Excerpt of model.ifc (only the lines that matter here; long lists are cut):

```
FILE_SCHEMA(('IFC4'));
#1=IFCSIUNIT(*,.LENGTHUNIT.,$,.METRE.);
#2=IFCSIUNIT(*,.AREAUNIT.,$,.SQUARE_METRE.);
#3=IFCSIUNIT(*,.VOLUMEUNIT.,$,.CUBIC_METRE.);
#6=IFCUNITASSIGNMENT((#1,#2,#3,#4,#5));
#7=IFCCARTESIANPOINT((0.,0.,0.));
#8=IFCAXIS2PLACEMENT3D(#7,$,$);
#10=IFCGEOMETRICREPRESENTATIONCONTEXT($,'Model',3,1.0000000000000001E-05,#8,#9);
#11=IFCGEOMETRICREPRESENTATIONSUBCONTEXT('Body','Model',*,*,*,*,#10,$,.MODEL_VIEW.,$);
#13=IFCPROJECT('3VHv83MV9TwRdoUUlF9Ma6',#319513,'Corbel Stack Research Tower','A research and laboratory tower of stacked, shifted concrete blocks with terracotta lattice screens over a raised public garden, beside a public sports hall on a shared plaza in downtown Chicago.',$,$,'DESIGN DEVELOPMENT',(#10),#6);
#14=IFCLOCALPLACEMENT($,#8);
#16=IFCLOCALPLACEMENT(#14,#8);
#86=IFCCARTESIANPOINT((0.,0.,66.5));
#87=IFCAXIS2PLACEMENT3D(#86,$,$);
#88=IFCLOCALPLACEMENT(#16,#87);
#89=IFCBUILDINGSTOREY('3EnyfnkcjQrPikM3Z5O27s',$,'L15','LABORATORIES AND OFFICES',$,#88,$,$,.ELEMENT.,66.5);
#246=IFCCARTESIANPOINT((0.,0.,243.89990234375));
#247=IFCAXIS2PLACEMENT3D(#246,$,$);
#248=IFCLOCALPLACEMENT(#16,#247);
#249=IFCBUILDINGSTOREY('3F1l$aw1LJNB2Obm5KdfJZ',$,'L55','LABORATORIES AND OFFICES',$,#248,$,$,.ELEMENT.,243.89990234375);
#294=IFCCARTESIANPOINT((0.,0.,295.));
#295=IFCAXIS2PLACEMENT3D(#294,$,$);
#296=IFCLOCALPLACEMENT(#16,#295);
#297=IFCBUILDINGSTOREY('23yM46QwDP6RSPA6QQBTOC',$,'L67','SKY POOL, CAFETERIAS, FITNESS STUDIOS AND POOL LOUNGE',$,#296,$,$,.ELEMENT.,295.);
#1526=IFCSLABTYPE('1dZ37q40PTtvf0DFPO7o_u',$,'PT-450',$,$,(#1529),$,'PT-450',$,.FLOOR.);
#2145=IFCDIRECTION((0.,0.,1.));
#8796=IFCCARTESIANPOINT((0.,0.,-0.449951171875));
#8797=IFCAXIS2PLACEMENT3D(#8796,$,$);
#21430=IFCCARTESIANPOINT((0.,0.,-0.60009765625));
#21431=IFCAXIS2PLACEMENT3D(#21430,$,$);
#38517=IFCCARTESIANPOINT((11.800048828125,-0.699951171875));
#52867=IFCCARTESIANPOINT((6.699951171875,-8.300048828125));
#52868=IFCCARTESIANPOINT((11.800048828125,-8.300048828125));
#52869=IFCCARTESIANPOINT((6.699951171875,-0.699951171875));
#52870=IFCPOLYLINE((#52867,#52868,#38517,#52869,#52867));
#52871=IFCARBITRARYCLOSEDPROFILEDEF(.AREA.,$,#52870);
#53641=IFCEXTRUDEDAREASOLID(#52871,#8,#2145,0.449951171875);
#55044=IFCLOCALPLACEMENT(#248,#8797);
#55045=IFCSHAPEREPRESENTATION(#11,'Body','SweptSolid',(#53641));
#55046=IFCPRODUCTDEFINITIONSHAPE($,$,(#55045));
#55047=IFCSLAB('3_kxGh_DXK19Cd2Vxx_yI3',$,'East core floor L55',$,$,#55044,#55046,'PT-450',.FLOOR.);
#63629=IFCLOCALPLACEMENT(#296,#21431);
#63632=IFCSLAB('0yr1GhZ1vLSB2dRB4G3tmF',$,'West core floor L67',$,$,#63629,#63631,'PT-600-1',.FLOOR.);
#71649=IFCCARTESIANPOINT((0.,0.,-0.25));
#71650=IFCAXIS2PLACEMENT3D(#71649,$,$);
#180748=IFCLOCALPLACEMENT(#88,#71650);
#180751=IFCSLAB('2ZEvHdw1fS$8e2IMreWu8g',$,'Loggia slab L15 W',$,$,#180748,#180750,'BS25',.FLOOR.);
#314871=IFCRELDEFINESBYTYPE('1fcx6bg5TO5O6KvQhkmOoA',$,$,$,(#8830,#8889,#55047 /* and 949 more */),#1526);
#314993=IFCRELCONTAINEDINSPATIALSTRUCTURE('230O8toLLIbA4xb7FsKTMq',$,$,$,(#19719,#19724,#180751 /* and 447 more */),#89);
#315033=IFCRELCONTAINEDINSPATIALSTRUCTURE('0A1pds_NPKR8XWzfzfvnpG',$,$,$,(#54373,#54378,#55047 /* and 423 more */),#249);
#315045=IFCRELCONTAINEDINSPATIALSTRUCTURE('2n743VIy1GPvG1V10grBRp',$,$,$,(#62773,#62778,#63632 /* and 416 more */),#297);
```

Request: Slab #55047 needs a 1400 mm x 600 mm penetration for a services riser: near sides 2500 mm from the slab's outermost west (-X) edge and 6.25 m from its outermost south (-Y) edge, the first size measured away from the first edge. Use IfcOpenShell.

```python
import numpy as np
import ifcopenshell
import ifcopenshell.api.feature
import ifcopenshell.api.geometry
import ifcopenshell.api.root
import ifcopenshell.geom
import ifcopenshell.util.placement
import ifcopenshell.util.representation
import ifcopenshell.util.shape
import ifcopenshell.util.unit

model = ifcopenshell.open("model.ifc")
unit_scale = ifcopenshell.util.unit.calculate_unit_scale(model)
settings = ifcopenshell.geom.settings()


def volume(element):
    """Net volume in cubic metres, openings subtracted."""
    shape = ifcopenshell.geom.create_shape(settings, element)
    return ifcopenshell.util.shape.get_volume(shape.geometry)


slab = model.by_guid("3_kxGh_DXK19Cd2Vxx_yI3")
before = volume(slab)

# Extent in the slab's own axes, in metres. The edges named are its -X and -Y sides.
slab_shape = ifcopenshell.geom.create_shape(settings, slab)
vertices = ifcopenshell.util.shape.get_vertices(slab_shape.geometry)
x_min, y_min, bottom = vertices.min(axis=0)
top = vertices[:, 2].max()

opening = ifcopenshell.api.root.create_entity(model, ifc_class="IfcOpeningElement", name="Services riser opening", predefined_type="OPENING")
context = ifcopenshell.util.representation.get_context(model, "Model", "Body", "MODEL_VIEW")
width, depth = 1.4, 0.6
outline = [(0.0, 0.0), (width, 0.0), (width, depth), (0.0, depth), (0.0, 0.0)]
# Overshoot both faces by 50 mm so the cut is clean.
shape = ifcopenshell.api.geometry.add_slab_representation(
    model, context=context, depth=top - bottom + 0.1, polyline=outline
)
ifcopenshell.api.geometry.assign_representation(model, product=opening, representation=shape)

matrix = ifcopenshell.util.placement.get_local_placement(slab.ObjectPlacement)
matrix[:, 3] = matrix @ np.append(np.array([x_min + 2.5, y_min + 6.25, bottom - 0.05]) / unit_scale, 1.0)
ifcopenshell.api.geometry.edit_object_placement(model, product=opening, matrix=matrix, is_si=False)
ifcopenshell.api.feature.add_feature(model, feature=opening, element=slab)

after = volume(slab)

print(f"slab volume {before:.3f} -> {after:.3f} m3")

model.write("model-out.ifc")
```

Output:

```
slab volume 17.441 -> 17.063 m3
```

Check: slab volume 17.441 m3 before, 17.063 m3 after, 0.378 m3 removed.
